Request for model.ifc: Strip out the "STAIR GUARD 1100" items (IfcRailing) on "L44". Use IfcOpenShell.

First a look at what the model holds.

```python
import ifcopenshell
import ifcopenshell.util.element

model = ifcopenshell.open("model.ifc")
print(model.schema)
storey = next(s for s in model.by_type("IfcBuildingStorey") if s.Name == "L44")
railings = [e for e in ifcopenshell.util.element.get_decomposition(storey) if e.is_a("IfcRailing")]
seen = {}
for e in railings:
    element_type = ifcopenshell.util.element.get_type(e)
    name = element_type.Name if element_type not in (None, e) else None
    seen[name] = seen.get(name, 0) + 1
for name, count in sorted(seen.items(), key=str):
    print(count, "x", name)
```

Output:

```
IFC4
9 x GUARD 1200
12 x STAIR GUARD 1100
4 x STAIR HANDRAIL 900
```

```python
import ifcopenshell
import ifcopenshell.api.root
import ifcopenshell.util.element

model = ifcopenshell.open("model.ifc")

storey = next(s for s in model.by_type("IfcBuildingStorey") if s.Name == "L44")
railings = [e for e in ifcopenshell.util.element.get_decomposition(storey) if e.is_a("IfcRailing")]
targets = [e for e in railings if (t := ifcopenshell.util.element.get_type(e)) not in (None, e) and t.Name == "STAIR GUARD 1100"]

for e in targets:
    ifcopenshell.api.root.remove_product(model, product=e)
print(len(targets), "removed")

model.write("model_rev.ifc")
```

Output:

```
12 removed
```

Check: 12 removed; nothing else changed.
